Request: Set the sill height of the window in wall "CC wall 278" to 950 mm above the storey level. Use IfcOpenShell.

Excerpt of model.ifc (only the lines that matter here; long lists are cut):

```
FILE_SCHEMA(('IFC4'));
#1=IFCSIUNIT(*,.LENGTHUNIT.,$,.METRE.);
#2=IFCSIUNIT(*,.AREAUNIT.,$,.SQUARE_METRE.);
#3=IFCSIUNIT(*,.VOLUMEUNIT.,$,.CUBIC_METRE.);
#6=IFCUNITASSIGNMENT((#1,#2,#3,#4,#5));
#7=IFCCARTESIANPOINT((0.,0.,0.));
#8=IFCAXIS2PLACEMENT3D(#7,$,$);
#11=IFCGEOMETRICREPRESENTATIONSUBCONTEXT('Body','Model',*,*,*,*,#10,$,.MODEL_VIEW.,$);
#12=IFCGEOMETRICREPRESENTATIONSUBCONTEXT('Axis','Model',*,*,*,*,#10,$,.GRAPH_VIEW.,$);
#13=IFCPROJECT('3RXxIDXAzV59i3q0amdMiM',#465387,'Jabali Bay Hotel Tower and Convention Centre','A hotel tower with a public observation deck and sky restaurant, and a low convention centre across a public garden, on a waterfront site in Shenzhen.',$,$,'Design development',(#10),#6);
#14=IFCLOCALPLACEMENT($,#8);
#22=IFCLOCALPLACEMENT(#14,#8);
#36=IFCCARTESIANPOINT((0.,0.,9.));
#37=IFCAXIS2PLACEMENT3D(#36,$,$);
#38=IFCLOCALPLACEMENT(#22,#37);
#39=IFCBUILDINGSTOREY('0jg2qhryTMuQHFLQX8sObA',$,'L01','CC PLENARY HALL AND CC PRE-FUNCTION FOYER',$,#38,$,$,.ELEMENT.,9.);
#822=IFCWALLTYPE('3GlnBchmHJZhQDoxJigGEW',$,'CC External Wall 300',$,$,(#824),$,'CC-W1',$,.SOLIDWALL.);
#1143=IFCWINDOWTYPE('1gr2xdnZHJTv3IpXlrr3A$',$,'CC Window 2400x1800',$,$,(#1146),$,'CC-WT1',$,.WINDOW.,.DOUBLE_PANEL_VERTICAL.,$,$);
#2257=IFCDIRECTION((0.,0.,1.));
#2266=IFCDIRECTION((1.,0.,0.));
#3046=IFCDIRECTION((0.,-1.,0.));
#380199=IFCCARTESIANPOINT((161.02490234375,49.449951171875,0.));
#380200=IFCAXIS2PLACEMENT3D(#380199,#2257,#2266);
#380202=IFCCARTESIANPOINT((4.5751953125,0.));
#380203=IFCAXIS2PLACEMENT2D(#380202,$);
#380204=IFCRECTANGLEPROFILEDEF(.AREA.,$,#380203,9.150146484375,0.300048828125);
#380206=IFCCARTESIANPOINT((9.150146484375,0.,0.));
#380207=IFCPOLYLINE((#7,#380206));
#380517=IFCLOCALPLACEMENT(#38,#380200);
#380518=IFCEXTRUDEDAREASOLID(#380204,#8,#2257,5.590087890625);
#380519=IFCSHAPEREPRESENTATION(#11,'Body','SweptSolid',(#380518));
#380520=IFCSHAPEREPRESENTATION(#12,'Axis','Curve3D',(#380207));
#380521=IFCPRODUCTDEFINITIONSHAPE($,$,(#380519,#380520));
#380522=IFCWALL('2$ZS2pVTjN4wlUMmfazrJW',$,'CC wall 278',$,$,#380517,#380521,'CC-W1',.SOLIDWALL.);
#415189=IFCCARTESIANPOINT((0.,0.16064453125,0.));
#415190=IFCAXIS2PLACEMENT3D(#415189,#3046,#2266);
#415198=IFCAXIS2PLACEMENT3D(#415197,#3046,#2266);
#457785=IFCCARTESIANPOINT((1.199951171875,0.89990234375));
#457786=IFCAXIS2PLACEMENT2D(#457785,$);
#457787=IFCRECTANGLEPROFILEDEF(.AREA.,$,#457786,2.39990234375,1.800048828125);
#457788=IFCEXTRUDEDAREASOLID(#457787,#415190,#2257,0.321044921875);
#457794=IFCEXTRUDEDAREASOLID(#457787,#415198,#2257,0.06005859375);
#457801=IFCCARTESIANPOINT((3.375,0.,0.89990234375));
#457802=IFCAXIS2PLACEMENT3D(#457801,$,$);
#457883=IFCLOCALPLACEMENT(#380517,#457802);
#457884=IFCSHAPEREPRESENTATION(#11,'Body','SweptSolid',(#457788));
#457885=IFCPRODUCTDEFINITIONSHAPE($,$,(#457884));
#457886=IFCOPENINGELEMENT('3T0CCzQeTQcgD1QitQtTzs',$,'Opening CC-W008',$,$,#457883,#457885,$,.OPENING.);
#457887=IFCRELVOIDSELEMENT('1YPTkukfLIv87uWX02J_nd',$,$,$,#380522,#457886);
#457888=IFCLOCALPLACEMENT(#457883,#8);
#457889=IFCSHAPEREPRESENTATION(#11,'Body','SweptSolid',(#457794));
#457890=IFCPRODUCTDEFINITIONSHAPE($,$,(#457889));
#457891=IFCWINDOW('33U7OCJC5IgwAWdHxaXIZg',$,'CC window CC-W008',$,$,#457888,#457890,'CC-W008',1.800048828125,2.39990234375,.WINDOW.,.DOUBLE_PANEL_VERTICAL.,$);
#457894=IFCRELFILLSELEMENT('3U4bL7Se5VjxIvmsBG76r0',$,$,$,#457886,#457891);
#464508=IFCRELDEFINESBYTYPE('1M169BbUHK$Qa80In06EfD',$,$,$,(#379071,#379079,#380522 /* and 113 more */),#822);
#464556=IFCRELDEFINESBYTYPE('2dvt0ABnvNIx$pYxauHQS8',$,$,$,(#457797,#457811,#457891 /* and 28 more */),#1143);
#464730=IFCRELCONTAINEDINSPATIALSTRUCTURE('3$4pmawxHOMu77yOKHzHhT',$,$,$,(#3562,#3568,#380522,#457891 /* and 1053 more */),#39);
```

```python
import numpy as np
import ifcopenshell
import ifcopenshell.api.geometry
import ifcopenshell.geom
import ifcopenshell.util.element
import ifcopenshell.util.placement
import ifcopenshell.util.shape
import ifcopenshell.util.unit

model = ifcopenshell.open("model.ifc")
unit_scale = ifcopenshell.util.unit.calculate_unit_scale(model)

window = model.by_id(457891)
opening = window.FillsVoids[0].RelatingOpeningElement
storey = ifcopenshell.util.element.get_container(window, ifc_class="IfcBuildingStorey")
level = ifcopenshell.util.placement.get_local_placement(storey.ObjectPlacement)[2, 3]

# The opening's origin need not be at the sill, so measure its lowest point.
shape = ifcopenshell.geom.create_shape(ifcopenshell.geom.settings(), opening)
bottom = ifcopenshell.util.shape.get_shape_bottom_elevation(shape, shape.geometry) / unit_scale
dz = level + 0.95 - bottom

shift = np.array([0.0, 0.0, dz])
# The window is placed relative to its opening, so it follows when the opening moves.
matrix = ifcopenshell.util.placement.get_local_placement(opening.ObjectPlacement)
matrix[:3, 3] += shift
ifcopenshell.api.geometry.edit_object_placement(
    model, product=opening, matrix=matrix, is_si=False, should_transform_children=True
)

print(f"moved by {dz * unit_scale:+.3f} m")

model.write("model_updated.ifc")
```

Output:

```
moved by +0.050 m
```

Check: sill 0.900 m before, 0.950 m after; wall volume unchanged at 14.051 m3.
